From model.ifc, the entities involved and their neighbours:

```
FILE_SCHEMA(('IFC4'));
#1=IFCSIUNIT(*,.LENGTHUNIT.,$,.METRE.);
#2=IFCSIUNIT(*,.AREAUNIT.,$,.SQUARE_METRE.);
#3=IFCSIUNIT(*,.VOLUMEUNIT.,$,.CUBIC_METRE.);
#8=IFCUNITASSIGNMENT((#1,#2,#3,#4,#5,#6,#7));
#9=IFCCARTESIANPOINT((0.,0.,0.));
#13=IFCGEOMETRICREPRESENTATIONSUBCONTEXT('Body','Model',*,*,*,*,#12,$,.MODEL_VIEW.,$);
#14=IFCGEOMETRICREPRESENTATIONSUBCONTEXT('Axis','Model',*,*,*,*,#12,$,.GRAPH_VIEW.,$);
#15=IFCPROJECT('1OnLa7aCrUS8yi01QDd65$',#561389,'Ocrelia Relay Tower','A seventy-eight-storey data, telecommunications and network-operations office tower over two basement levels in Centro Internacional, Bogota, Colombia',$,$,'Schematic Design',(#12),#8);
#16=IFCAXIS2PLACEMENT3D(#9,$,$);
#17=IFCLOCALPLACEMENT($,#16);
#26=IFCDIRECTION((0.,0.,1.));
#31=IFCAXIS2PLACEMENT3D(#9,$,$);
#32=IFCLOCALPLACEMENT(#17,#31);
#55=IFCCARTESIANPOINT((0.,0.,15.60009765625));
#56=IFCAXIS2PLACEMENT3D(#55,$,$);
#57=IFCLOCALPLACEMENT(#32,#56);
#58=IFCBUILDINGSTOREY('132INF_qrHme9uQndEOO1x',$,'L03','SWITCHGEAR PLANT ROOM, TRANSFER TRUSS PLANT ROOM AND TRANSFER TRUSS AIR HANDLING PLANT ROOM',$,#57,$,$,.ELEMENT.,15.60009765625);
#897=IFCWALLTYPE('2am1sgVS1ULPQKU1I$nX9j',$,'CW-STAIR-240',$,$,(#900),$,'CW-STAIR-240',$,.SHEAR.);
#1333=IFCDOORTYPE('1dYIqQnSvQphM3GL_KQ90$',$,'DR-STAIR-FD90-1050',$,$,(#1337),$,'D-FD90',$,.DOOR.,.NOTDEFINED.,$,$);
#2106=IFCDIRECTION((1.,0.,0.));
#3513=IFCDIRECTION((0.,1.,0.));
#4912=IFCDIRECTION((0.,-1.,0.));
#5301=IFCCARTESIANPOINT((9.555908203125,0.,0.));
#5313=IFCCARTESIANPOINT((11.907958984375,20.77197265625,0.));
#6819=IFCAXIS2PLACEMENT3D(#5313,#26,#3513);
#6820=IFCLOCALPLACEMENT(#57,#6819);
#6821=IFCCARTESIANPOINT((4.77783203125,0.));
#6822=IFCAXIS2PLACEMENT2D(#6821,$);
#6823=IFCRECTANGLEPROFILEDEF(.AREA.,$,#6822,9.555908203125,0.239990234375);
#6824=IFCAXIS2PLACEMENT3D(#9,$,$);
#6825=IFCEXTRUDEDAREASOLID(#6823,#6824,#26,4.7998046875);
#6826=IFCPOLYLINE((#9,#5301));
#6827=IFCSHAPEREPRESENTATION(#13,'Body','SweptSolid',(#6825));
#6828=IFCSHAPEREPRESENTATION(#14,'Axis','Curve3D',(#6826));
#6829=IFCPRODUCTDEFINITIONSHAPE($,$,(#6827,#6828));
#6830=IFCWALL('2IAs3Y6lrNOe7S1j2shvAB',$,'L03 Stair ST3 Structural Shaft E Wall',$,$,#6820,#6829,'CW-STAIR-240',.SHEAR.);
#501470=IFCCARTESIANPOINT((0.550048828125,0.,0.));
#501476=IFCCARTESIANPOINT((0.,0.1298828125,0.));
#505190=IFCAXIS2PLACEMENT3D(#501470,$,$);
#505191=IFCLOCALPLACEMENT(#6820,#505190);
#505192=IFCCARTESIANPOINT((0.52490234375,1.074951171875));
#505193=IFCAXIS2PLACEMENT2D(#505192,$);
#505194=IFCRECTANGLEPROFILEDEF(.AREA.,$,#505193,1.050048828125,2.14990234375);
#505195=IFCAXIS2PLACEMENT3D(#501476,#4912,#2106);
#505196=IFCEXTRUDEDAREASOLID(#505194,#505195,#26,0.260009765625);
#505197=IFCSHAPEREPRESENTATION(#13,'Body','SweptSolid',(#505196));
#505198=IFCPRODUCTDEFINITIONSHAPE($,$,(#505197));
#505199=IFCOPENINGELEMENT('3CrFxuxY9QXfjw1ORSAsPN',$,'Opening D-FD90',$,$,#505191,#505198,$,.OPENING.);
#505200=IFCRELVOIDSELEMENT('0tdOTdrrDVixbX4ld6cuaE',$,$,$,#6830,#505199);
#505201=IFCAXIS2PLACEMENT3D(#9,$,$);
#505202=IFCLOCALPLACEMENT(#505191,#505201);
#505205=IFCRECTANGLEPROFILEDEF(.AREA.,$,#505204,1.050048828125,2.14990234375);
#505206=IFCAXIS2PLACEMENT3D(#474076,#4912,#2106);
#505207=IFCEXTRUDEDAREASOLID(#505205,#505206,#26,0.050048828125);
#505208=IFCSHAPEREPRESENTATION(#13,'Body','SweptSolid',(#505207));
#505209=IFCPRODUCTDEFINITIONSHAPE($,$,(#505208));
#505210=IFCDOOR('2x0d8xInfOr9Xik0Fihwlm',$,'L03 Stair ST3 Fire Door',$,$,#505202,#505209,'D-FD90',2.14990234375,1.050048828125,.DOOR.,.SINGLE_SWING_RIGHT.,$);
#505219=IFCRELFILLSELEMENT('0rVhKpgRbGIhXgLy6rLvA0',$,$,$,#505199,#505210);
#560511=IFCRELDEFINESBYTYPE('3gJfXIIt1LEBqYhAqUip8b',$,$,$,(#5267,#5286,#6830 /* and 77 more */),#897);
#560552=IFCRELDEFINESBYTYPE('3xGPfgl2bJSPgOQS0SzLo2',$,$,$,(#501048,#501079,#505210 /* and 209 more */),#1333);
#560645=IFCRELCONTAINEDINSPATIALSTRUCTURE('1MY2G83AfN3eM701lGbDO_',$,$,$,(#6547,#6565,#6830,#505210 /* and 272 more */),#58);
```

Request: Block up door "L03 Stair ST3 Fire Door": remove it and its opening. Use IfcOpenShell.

```python
import ifcopenshell
import ifcopenshell.api.feature
import ifcopenshell.api.root
import ifcopenshell.geom
import ifcopenshell.util.shape

model = ifcopenshell.open("model.ifc")
settings = ifcopenshell.geom.settings()


def volume(element):
    """Net volume in cubic metres, openings subtracted."""
    shape = ifcopenshell.geom.create_shape(settings, element)
    return ifcopenshell.util.shape.get_volume(shape.geometry)


door = model.by_guid("2x0d8xInfOr9Xik0Fihwlm")
opening = door.FillsVoids[0].RelatingOpeningElement
wall = opening.VoidsElements[0].RelatingBuildingElement
before = volume(wall)

ifcopenshell.api.root.remove_product(model, product=door)
ifcopenshell.api.feature.remove_feature(model, feature=opening)

after = volume(wall)

print(f"wall volume {before:.3f} -> {after:.3f} m3")

model.write("model_updated.ifc")
```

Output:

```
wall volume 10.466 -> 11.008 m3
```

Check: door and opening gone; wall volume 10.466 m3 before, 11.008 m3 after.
